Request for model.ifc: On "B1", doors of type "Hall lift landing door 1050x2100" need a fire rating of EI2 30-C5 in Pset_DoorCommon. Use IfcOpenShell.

First a look at what the model holds.

```python
import ifcopenshell
import ifcopenshell.util.element

model = ifcopenshell.open("model.ifc")
print(model.schema)
storey = next(s for s in model.by_type("IfcBuildingStorey") if s.Name == "B1")
doors = [e for e in ifcopenshell.util.element.get_decomposition(storey) if e.is_a("IfcDoor")]
seen = {}
for e in doors:
    element_type = ifcopenshell.util.element.get_type(e)
    key = (element_type.Name if element_type != e and element_type else None, ifcopenshell.util.element.get_pset(e, "Pset_DoorCommon", "FireRating"))
    seen[key] = seen.get(key, 0) + 1
for (name, value), count in sorted(seen.items(), key=str):
    print(count, "x", name, "|", value)
```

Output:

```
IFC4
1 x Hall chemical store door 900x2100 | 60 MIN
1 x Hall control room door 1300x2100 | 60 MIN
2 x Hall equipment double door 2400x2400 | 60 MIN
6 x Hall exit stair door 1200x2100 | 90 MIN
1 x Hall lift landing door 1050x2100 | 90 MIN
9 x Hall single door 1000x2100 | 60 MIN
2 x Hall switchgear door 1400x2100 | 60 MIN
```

```python
import ifcopenshell
import ifcopenshell.api.pset
import ifcopenshell.util.element

model = ifcopenshell.open("model.ifc")

storey = next(s for s in model.by_type("IfcBuildingStorey") if s.Name == "B1")
doors = [e for e in ifcopenshell.util.element.get_decomposition(storey) if e.is_a("IfcDoor")]

count = 0
for e in doors:
    element_type = ifcopenshell.util.element.get_type(e)
    if element_type in (None, e) or element_type.Name != "Hall lift landing door 1050x2100":
        continue
    # add_pset returns the element's existing set when there is one.
    pset = ifcopenshell.api.pset.add_pset(model, product=e, name="Pset_DoorCommon")
    ifcopenshell.api.pset.edit_pset(model, pset=pset, properties={"FireRating": "EI2 30-C5"})
    count += 1

print(count, "doors updated")

model.write("model_v2.ifc")
```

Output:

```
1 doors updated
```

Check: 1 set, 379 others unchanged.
